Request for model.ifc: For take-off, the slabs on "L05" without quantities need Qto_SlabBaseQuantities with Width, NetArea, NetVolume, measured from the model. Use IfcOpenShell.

First a look at what the model holds.

```python
import ifcopenshell
import ifcopenshell.util.element
import ifcopenshell.util.unit

model = ifcopenshell.open("model.ifc")
print(model.schema)
for unit_type in ("LENGTHUNIT", "AREAUNIT", "VOLUMEUNIT"):
    print(unit_type, ifcopenshell.util.unit.calculate_unit_scale(model, unit_type))
storey = next(s for s in model.by_type("IfcBuildingStorey") if s.Name == "L05")
slabs = [e for e in ifcopenshell.util.element.get_decomposition(storey) if e.is_a("IfcSlab")]
for e in sorted(slabs, key=lambda e: e.id()):
    print(e.id(), e.is_a(), e.Name, list(ifcopenshell.util.element.get_psets(e, qtos_only=True)), sep=" | ")
```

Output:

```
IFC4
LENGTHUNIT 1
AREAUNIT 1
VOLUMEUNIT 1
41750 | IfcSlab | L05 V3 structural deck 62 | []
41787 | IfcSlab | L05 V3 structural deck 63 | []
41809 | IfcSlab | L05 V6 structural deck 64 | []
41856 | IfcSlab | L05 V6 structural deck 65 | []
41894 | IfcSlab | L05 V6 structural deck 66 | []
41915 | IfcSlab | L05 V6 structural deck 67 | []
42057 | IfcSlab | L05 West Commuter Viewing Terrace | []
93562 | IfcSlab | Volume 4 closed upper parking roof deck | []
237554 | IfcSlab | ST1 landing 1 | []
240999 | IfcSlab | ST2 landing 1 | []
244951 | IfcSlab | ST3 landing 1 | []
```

```python
import ifcopenshell
import ifcopenshell.api.pset
import ifcopenshell.geom
import ifcopenshell.util.element
import ifcopenshell.util.shape
import ifcopenshell.util.unit

model = ifcopenshell.open("model.ifc")
unit_scale = ifcopenshell.util.unit.calculate_unit_scale(model)
area_scale = ifcopenshell.util.unit.calculate_unit_scale(model, "AREAUNIT")
volume_scale = ifcopenshell.util.unit.calculate_unit_scale(model, "VOLUMEUNIT")
settings = ifcopenshell.geom.settings()

storey = next(s for s in model.by_type("IfcBuildingStorey") if s.Name == "L05")
slabs = [e for e in ifcopenshell.util.element.get_decomposition(storey) if e.is_a("IfcSlab")]

for e in sorted(slabs, key=lambda e: e.id()):
    if ifcopenshell.util.element.get_psets(e, qtos_only=True, should_inherit=False):
        continue
    # Geometry comes back in metres, in the element's own axes.
    shape = ifcopenshell.geom.create_shape(settings, e)
    values = {
        "Width": ifcopenshell.util.shape.get_z(shape.geometry) / unit_scale,
        "NetArea": ifcopenshell.util.shape.get_footprint_area(shape.geometry) / area_scale,
        "NetVolume": ifcopenshell.util.shape.get_volume(shape.geometry) / volume_scale,
    }
    qto = ifcopenshell.api.pset.add_qto(model, product=e, name="Qto_SlabBaseQuantities")
    ifcopenshell.api.pset.edit_qto(model, qto=qto, properties=values)
    print(e.id(), {k: round(v, 3) for k, v in values.items()})

model.write("model_v2.ifc")
```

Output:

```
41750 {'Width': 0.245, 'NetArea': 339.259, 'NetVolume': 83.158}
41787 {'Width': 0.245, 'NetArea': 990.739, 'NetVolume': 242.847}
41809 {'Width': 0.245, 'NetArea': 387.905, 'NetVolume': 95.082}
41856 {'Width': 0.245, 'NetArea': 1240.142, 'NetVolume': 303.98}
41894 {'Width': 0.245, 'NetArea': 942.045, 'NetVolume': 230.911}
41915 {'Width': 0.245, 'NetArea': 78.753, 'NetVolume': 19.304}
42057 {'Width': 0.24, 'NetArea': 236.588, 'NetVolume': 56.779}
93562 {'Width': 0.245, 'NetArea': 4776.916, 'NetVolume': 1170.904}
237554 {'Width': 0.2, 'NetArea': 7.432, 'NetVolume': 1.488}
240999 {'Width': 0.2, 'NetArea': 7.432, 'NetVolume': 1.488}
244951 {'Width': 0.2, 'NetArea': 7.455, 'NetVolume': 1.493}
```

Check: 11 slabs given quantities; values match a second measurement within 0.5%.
